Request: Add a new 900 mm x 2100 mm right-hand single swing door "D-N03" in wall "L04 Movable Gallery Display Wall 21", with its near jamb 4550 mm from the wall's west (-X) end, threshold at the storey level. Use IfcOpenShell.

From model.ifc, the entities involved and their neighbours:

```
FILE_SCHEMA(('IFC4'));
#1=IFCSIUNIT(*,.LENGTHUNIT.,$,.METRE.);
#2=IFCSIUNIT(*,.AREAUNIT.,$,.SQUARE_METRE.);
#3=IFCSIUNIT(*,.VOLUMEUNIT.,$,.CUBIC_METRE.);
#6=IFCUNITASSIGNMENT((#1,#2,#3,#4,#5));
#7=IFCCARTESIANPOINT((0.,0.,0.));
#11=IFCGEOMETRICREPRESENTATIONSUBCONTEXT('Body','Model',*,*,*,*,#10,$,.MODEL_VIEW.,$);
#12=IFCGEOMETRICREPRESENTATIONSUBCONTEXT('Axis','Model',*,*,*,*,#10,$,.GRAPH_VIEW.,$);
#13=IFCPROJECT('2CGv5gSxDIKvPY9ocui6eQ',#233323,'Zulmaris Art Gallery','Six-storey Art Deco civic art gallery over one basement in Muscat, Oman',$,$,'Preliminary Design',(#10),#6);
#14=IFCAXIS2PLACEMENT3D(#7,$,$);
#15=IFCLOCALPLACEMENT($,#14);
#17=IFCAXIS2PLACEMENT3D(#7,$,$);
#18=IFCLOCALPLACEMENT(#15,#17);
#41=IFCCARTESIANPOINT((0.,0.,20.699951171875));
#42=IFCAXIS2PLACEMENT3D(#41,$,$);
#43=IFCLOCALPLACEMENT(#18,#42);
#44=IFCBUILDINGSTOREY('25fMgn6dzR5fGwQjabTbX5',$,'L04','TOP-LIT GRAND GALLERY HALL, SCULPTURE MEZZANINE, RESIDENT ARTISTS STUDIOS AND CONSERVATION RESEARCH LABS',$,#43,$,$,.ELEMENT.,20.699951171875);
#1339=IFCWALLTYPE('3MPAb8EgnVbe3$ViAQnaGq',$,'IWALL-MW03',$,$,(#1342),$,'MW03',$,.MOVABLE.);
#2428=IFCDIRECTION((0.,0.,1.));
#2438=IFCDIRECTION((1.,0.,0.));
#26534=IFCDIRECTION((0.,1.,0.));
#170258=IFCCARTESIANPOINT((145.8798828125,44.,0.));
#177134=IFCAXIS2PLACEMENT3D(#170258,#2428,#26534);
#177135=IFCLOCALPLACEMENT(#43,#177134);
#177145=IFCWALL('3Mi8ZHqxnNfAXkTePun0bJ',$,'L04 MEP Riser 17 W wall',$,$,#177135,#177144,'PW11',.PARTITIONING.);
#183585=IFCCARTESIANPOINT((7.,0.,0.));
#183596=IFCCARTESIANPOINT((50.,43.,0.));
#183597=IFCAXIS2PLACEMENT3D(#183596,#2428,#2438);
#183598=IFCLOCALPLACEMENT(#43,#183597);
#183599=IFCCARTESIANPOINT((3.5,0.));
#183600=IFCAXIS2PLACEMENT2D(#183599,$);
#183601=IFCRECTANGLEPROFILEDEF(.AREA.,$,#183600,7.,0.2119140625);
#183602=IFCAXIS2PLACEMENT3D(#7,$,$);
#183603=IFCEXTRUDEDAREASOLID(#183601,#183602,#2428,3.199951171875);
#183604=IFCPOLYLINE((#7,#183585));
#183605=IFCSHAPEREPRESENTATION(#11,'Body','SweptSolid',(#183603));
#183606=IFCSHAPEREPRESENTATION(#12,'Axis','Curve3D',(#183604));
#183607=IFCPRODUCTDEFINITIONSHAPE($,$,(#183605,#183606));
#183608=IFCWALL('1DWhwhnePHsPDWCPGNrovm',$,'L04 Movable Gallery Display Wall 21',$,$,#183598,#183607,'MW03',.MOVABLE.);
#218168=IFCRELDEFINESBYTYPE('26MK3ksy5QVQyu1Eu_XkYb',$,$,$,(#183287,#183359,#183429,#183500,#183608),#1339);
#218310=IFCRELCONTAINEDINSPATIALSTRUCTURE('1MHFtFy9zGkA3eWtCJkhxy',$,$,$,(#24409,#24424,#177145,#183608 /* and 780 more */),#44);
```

```python
import numpy as np
import ifcopenshell
import ifcopenshell.api.feature
import ifcopenshell.api.geometry
import ifcopenshell.api.root
import ifcopenshell.api.spatial
import ifcopenshell.geom
import ifcopenshell.util.element
import ifcopenshell.util.placement
import ifcopenshell.util.representation
import ifcopenshell.util.shape
import ifcopenshell.util.unit

model = ifcopenshell.open("model.ifc")
unit_scale = ifcopenshell.util.unit.calculate_unit_scale(model)
settings = ifcopenshell.geom.settings()


def volume(element):
    """Net volume in cubic metres, openings subtracted."""
    shape = ifcopenshell.geom.create_shape(settings, element)
    return ifcopenshell.util.shape.get_volume(shape.geometry)


wall = model.by_guid("1DWhwhnePHsPDWCPGNrovm")
storey = ifcopenshell.util.element.get_container(wall, ifc_class="IfcBuildingStorey")
context = ifcopenshell.util.representation.get_context(model, "Model", "Body", "MODEL_VIEW")
before = volume(wall)

width, height, from_end, sill = 0.9, 2.1, 4.55, 0.0  # metres

# The wall runs along its own X axis, and the end named is its -X end.
wall_shape = ifcopenshell.geom.create_shape(settings, wall)
x, y, z = ifcopenshell.util.shape.get_vertices(wall_shape.geometry).T
start = x.min() + from_end
face, thickness = float(y.min()), float(y.max() - y.min())
wall_matrix = ifcopenshell.util.placement.get_local_placement(wall.ObjectPlacement)
level = ifcopenshell.util.placement.get_local_placement(storey.ObjectPlacement)[2, 3]


def in_wall(x, y):
    """Placement at x, y metres in the wall's axes, at sill height."""
    matrix = wall_matrix.copy()
    matrix[:, 3] = wall_matrix @ np.array([x / unit_scale, y / unit_scale, 0.0, 1.0])
    matrix[2, 3] = level + sill / unit_scale
    return matrix


# Opening: a box that overshoots both wall faces by 50 mm.
opening = ifcopenshell.api.root.create_entity(model, ifc_class="IfcOpeningElement", predefined_type="OPENING")
box = ifcopenshell.api.geometry.add_wall_representation(
    model, context=context, length=width, height=height, thickness=thickness + 0.1
)
ifcopenshell.api.geometry.assign_representation(model, product=opening, representation=box)
ifcopenshell.api.geometry.edit_object_placement(model, product=opening, matrix=in_wall(start, face - 0.05), is_si=False)
ifcopenshell.api.feature.add_feature(model, feature=opening, element=wall)

door = ifcopenshell.api.root.create_entity(model, ifc_class="IfcDoor", name="D-N03", predefined_type="DOOR")
door.OverallWidth, door.OverallHeight = width / unit_scale, height / unit_scale
door.OperationType = "SINGLE_SWING_RIGHT"
body = ifcopenshell.api.geometry.add_door_representation(
    model,
    context=context,
    overall_width=door.OverallWidth,
    overall_height=door.OverallHeight,
    operation_type="SINGLE_SWING_RIGHT",
    lining_properties={"LiningDepth": thickness / unit_scale, "ThresholdDepth": thickness / unit_scale},
)
ifcopenshell.api.geometry.assign_representation(model, product=door, representation=body)
ifcopenshell.api.spatial.assign_container(model, products=[door], relating_structure=storey)
ifcopenshell.api.feature.add_filling(model, opening=opening, element=door)

# The lining spans the wall, so the door starts at the wall face.
ifcopenshell.api.geometry.edit_object_placement(model, product=door, matrix=in_wall(start, face), is_si=False)

after = volume(wall)

print(f"wall volume {before:.3f} -> {after:.3f} m3")

model.write("model_updated.ifc")
```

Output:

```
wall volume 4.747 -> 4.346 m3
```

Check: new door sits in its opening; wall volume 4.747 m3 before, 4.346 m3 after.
